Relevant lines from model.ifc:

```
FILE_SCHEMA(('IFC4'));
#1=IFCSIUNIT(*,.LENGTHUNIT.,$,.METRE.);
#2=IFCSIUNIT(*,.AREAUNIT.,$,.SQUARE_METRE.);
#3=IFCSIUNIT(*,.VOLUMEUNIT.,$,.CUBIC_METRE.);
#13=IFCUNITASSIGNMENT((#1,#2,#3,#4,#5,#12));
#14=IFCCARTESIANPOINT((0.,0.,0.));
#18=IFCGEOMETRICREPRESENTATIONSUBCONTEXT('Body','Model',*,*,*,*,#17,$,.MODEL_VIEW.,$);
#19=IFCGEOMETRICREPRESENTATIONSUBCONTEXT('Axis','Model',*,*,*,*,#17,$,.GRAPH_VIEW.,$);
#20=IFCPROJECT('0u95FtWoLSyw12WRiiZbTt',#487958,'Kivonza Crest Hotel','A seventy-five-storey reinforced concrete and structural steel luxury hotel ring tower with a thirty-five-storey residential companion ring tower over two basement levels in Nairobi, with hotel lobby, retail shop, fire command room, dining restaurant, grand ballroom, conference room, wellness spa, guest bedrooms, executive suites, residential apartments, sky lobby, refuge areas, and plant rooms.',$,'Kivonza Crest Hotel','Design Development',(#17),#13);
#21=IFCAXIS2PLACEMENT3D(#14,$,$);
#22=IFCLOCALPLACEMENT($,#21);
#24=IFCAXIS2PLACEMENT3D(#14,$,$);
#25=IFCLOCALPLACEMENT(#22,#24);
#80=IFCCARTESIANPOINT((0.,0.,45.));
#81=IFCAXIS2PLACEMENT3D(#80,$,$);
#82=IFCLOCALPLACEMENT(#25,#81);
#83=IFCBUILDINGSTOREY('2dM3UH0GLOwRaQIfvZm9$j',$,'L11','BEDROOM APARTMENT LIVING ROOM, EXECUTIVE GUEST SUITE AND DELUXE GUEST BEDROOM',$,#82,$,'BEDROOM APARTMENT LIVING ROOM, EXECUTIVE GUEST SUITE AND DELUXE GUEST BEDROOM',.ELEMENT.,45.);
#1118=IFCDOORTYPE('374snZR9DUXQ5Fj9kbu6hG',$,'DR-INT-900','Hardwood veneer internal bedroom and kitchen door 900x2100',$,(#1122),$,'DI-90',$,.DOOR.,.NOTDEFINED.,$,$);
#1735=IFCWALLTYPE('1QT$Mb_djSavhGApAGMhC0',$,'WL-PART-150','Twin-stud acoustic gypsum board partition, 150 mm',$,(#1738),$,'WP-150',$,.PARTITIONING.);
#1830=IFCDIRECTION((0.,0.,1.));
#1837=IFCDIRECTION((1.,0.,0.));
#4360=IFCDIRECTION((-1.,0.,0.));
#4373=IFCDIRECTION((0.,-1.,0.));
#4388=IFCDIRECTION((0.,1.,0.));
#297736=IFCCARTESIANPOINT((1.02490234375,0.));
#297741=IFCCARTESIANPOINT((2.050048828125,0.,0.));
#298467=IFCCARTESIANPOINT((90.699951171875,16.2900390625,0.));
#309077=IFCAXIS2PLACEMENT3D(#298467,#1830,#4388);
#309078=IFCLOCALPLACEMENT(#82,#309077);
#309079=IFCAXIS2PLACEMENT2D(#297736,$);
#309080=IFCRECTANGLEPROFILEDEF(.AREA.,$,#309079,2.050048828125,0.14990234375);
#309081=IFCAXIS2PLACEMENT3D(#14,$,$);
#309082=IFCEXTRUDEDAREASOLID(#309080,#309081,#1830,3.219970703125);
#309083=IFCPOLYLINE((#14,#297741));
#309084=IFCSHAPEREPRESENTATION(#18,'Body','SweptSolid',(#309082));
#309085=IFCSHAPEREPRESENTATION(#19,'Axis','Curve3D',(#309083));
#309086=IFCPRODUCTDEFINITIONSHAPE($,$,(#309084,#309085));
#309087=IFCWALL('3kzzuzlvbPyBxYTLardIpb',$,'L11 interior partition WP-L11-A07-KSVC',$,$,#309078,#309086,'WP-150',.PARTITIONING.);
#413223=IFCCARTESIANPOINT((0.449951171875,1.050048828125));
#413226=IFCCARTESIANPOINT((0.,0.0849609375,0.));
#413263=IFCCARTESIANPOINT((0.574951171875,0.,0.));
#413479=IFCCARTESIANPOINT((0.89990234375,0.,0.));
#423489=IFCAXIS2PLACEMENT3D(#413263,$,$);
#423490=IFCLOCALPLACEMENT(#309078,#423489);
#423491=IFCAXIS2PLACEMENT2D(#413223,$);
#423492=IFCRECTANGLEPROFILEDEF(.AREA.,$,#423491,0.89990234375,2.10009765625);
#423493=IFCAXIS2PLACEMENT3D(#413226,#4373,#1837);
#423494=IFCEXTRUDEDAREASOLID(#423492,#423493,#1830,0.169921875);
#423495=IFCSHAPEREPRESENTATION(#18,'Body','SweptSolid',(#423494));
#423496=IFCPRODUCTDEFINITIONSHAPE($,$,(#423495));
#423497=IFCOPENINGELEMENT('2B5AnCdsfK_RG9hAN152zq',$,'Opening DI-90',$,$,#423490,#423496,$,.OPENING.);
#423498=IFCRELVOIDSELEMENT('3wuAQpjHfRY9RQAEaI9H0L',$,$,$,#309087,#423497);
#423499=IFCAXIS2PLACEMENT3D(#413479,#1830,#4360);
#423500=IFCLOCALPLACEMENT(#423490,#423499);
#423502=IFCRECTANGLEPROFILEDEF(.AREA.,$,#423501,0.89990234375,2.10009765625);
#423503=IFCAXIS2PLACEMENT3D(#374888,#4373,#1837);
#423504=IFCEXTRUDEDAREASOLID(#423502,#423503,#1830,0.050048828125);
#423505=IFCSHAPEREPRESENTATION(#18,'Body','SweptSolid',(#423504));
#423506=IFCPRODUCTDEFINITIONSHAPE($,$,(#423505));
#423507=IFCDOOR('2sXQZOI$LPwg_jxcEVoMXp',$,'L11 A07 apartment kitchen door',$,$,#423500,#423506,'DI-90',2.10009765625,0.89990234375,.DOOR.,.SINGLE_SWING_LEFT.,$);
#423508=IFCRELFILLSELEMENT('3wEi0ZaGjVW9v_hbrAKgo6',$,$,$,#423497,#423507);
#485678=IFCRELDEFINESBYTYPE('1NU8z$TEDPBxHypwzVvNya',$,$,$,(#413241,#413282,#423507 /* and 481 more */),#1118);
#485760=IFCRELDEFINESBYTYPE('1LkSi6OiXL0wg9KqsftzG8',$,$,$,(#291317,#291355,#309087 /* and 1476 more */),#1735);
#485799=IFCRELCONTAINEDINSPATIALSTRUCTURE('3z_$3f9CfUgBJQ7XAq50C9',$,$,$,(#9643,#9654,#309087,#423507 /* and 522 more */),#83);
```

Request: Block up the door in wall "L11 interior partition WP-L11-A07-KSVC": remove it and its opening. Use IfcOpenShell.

```python
import ifcopenshell
import ifcopenshell.api.feature
import ifcopenshell.api.root
import ifcopenshell.geom
import ifcopenshell.util.shape

model = ifcopenshell.open("model.ifc")
settings = ifcopenshell.geom.settings()


def volume(element):
    """Net volume in cubic metres, openings subtracted."""
    shape = ifcopenshell.geom.create_shape(settings, element)
    return ifcopenshell.util.shape.get_volume(shape.geometry)


door = model.by_guid("2sXQZOI$LPwg_jxcEVoMXp")
opening = door.FillsVoids[0].RelatingOpeningElement
wall = opening.VoidsElements[0].RelatingBuildingElement
before = volume(wall)

ifcopenshell.api.root.remove_product(model, product=door)
ifcopenshell.api.feature.remove_feature(model, feature=opening)

after = volume(wall)

print(f"wall volume {before:.3f} -> {after:.3f} m3")

model.write("model_rev.ifc")
```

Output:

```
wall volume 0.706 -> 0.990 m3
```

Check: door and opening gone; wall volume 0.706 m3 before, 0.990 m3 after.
